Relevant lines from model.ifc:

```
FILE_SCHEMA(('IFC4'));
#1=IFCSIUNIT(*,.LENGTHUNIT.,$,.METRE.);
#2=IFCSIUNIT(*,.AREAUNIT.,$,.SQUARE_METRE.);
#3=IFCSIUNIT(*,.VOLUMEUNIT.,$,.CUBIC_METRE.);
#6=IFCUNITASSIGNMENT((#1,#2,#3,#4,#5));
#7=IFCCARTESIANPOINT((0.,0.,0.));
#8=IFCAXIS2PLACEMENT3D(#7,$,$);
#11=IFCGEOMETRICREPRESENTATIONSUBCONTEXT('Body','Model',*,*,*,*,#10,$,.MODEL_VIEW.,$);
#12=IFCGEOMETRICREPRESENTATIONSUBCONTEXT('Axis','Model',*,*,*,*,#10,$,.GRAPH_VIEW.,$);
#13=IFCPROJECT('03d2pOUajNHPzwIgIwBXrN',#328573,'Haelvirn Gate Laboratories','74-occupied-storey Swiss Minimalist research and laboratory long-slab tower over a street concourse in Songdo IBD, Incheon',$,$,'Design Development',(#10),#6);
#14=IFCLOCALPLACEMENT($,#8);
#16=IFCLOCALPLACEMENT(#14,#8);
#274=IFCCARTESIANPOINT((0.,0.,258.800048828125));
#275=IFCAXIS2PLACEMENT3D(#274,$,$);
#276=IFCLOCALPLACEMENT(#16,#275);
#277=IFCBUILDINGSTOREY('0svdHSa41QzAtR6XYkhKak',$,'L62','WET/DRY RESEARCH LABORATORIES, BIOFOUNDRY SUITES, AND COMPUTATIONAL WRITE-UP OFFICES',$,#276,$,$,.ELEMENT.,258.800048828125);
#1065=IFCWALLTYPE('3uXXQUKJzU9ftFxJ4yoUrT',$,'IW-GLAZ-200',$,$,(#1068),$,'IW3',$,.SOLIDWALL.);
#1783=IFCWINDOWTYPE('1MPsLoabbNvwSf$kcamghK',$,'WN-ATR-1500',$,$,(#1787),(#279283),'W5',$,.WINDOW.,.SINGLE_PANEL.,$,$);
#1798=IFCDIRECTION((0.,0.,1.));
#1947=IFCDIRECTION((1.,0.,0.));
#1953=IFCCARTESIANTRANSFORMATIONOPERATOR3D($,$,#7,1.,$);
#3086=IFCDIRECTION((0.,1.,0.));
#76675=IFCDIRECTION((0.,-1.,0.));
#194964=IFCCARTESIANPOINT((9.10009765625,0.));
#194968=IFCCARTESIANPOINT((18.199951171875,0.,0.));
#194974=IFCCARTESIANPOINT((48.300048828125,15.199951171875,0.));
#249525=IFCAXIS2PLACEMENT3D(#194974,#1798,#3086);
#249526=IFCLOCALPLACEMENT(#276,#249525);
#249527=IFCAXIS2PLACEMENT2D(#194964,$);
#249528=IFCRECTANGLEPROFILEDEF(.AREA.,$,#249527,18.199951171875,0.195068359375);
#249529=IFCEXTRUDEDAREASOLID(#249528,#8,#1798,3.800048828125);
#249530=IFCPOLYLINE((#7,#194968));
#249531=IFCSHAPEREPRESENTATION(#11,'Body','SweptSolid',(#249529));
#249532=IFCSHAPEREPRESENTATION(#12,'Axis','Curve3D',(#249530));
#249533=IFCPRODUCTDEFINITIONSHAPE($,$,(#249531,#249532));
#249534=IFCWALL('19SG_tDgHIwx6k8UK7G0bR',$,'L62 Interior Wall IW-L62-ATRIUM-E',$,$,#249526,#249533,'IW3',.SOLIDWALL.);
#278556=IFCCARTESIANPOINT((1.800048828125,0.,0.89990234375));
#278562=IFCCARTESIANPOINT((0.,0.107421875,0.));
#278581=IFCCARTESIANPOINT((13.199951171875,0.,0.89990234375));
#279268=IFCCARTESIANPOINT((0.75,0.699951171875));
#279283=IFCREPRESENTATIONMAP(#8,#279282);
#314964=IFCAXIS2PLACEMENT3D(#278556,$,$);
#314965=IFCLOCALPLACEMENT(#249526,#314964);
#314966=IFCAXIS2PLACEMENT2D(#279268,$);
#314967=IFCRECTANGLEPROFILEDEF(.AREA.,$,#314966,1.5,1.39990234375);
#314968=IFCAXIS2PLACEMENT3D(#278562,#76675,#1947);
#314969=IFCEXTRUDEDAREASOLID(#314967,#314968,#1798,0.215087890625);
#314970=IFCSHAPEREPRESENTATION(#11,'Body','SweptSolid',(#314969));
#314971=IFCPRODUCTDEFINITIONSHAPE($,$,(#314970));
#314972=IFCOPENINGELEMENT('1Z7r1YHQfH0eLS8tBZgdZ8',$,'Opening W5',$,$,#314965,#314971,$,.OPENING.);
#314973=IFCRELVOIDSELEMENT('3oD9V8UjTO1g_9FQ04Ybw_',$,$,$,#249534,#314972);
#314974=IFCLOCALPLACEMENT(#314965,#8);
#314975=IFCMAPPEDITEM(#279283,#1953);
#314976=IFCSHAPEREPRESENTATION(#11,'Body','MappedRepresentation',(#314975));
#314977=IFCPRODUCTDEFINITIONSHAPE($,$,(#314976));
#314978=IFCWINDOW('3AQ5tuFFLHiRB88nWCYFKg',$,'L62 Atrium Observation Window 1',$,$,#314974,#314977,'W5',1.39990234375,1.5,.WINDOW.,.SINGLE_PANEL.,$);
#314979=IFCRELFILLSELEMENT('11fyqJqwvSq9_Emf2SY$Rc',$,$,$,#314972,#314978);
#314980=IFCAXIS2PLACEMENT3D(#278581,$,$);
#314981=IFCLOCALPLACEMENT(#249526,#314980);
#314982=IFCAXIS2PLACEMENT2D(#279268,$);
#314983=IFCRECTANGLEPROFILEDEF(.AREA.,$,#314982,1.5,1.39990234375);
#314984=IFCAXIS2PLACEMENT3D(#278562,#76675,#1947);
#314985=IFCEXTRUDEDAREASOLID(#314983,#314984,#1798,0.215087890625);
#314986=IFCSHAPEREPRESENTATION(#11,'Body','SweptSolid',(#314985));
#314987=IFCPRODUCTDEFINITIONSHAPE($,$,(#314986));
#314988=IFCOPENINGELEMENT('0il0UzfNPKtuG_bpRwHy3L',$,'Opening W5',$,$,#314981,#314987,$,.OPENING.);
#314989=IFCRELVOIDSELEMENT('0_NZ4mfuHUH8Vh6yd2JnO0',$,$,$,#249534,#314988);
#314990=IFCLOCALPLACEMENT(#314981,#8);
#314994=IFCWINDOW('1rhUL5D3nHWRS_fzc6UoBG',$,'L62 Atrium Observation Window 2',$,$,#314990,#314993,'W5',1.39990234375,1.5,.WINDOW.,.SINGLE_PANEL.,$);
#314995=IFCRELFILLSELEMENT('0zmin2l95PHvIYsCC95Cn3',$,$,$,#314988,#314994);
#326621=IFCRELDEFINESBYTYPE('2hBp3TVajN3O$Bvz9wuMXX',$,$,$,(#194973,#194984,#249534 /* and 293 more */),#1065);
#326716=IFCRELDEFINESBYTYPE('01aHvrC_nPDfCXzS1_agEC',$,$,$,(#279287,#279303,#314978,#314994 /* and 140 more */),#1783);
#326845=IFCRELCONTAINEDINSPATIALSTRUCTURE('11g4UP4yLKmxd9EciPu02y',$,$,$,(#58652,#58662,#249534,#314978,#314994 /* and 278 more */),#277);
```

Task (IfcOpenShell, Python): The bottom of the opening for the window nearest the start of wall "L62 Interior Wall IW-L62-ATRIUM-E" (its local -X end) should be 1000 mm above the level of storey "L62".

```python
import numpy as np
import ifcopenshell
import ifcopenshell.api.geometry
import ifcopenshell.geom
import ifcopenshell.util.element
import ifcopenshell.util.placement
import ifcopenshell.util.shape
import ifcopenshell.util.unit

model = ifcopenshell.open("model.ifc")
unit_scale = ifcopenshell.util.unit.calculate_unit_scale(model)

window = model.by_guid("3AQ5tuFFLHiRB88nWCYFKg")
opening = window.FillsVoids[0].RelatingOpeningElement
storey = ifcopenshell.util.element.get_container(window, ifc_class="IfcBuildingStorey")
level = ifcopenshell.util.placement.get_local_placement(storey.ObjectPlacement)[2, 3]

# The opening's origin need not be at the sill, so measure its lowest point.
shape = ifcopenshell.geom.create_shape(ifcopenshell.geom.settings(), opening)
bottom = ifcopenshell.util.shape.get_shape_bottom_elevation(shape, shape.geometry) / unit_scale
dz = level + 1 / unit_scale - bottom

shift = np.array([0.0, 0.0, dz])
# The window is placed relative to its opening, so it follows when the opening moves.
matrix = ifcopenshell.util.placement.get_local_placement(opening.ObjectPlacement)
matrix[:3, 3] += shift
ifcopenshell.api.geometry.edit_object_placement(
    model, product=opening, matrix=matrix, is_si=False, should_transform_children=True
)

print(f"moved by {dz * unit_scale:+.3f} m")

model.write("model_updated.ifc")
```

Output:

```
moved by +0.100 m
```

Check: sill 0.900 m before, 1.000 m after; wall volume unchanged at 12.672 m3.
